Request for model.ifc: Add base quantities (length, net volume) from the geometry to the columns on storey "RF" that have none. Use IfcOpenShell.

First a look at what the model holds.

```python
import ifcopenshell
import ifcopenshell.util.element
import ifcopenshell.util.unit

model = ifcopenshell.open("model.ifc")
print(model.schema)
for unit_type in ("LENGTHUNIT", "AREAUNIT", "VOLUMEUNIT"):
    print(unit_type, ifcopenshell.util.unit.calculate_unit_scale(model, unit_type))
storey = next(s for s in model.by_type("IfcBuildingStorey") if s.Name == "RF")
columns = [e for e in ifcopenshell.util.element.get_decomposition(storey) if e.is_a("IfcColumn")]
for e in sorted(columns, key=lambda e: e.id()):
    print(e.id(), e.is_a(), e.Name, list(ifcopenshell.util.element.get_psets(e, qtos_only=True)), sep=" | ")
```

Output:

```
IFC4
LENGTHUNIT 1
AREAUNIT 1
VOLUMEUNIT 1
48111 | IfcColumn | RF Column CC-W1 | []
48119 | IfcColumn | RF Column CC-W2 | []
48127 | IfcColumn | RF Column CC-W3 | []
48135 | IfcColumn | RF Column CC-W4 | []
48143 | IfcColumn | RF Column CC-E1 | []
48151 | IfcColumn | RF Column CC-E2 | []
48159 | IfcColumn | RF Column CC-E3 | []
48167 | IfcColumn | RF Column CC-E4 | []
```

```python
import ifcopenshell
import ifcopenshell.api.pset
import ifcopenshell.geom
import ifcopenshell.util.element
import ifcopenshell.util.shape
import ifcopenshell.util.unit

model = ifcopenshell.open("model.ifc")
unit_scale = ifcopenshell.util.unit.calculate_unit_scale(model)
volume_scale = ifcopenshell.util.unit.calculate_unit_scale(model, "VOLUMEUNIT")
settings = ifcopenshell.geom.settings()

storey = next(s for s in model.by_type("IfcBuildingStorey") if s.Name == "RF")
columns = [e for e in ifcopenshell.util.element.get_decomposition(storey) if e.is_a("IfcColumn")]

for e in sorted(columns, key=lambda e: e.id()):
    if ifcopenshell.util.element.get_psets(e, qtos_only=True, should_inherit=False):
        continue
    # Geometry comes back in metres, in the element's own axes.
    shape = ifcopenshell.geom.create_shape(settings, e)
    values = {
        "Length": ifcopenshell.util.shape.get_z(shape.geometry) / unit_scale,
        "NetVolume": ifcopenshell.util.shape.get_volume(shape.geometry) / volume_scale,
    }
    qto = ifcopenshell.api.pset.add_qto(model, product=e, name="Qto_ColumnBaseQuantities")
    ifcopenshell.api.pset.edit_qto(model, qto=qto, properties=values)
    print(e.id(), {k: round(v, 3) for k, v in values.items()})

model.write("model_v2.ifc")
```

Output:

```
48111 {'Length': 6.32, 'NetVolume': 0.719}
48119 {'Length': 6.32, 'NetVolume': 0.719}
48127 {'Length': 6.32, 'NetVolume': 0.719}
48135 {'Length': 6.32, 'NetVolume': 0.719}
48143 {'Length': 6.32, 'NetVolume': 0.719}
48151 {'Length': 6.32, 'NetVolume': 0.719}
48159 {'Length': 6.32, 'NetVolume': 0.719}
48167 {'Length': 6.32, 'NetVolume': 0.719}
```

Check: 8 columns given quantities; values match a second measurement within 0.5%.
